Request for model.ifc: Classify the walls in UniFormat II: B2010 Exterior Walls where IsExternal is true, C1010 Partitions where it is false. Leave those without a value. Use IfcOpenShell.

First a look at what the model holds.

```python
import ifcopenshell
import ifcopenshell.util.element

model = ifcopenshell.open("model.ifc")
print(model.schema)
print("classifications:", [c.Name for c in model.by_type("IfcClassification")])
values = [ifcopenshell.util.element.get_pset(e, "Pset_WallCommon", "IsExternal") for e in model.by_type("IfcWall")]
for value in (True, False, None):
    print("IsExternal", value, values.count(value))
```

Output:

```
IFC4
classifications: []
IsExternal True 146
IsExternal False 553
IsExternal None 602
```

```python
import ifcopenshell
import ifcopenshell.api.classification
import ifcopenshell.util.element

model = ifcopenshell.open("model.ifc")

system = ifcopenshell.api.classification.add_classification(model, classification="UniFormat II")

walls = model.by_type("IfcWall")
external = {e: ifcopenshell.util.element.get_pset(e, "Pset_WallCommon", "IsExternal") for e in walls}
for flag, code, name in ((True, "B2010", "Exterior Walls"), (False, "C1010", "Partitions")):
    products = [e for e in walls if external[e] is flag]
    ifcopenshell.api.classification.add_reference(
        model, products=products, classification=system, identification=code, name=name
    )
    print(code, len(products))

model.write("model_updated.ifc")
```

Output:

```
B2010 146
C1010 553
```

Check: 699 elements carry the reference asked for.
